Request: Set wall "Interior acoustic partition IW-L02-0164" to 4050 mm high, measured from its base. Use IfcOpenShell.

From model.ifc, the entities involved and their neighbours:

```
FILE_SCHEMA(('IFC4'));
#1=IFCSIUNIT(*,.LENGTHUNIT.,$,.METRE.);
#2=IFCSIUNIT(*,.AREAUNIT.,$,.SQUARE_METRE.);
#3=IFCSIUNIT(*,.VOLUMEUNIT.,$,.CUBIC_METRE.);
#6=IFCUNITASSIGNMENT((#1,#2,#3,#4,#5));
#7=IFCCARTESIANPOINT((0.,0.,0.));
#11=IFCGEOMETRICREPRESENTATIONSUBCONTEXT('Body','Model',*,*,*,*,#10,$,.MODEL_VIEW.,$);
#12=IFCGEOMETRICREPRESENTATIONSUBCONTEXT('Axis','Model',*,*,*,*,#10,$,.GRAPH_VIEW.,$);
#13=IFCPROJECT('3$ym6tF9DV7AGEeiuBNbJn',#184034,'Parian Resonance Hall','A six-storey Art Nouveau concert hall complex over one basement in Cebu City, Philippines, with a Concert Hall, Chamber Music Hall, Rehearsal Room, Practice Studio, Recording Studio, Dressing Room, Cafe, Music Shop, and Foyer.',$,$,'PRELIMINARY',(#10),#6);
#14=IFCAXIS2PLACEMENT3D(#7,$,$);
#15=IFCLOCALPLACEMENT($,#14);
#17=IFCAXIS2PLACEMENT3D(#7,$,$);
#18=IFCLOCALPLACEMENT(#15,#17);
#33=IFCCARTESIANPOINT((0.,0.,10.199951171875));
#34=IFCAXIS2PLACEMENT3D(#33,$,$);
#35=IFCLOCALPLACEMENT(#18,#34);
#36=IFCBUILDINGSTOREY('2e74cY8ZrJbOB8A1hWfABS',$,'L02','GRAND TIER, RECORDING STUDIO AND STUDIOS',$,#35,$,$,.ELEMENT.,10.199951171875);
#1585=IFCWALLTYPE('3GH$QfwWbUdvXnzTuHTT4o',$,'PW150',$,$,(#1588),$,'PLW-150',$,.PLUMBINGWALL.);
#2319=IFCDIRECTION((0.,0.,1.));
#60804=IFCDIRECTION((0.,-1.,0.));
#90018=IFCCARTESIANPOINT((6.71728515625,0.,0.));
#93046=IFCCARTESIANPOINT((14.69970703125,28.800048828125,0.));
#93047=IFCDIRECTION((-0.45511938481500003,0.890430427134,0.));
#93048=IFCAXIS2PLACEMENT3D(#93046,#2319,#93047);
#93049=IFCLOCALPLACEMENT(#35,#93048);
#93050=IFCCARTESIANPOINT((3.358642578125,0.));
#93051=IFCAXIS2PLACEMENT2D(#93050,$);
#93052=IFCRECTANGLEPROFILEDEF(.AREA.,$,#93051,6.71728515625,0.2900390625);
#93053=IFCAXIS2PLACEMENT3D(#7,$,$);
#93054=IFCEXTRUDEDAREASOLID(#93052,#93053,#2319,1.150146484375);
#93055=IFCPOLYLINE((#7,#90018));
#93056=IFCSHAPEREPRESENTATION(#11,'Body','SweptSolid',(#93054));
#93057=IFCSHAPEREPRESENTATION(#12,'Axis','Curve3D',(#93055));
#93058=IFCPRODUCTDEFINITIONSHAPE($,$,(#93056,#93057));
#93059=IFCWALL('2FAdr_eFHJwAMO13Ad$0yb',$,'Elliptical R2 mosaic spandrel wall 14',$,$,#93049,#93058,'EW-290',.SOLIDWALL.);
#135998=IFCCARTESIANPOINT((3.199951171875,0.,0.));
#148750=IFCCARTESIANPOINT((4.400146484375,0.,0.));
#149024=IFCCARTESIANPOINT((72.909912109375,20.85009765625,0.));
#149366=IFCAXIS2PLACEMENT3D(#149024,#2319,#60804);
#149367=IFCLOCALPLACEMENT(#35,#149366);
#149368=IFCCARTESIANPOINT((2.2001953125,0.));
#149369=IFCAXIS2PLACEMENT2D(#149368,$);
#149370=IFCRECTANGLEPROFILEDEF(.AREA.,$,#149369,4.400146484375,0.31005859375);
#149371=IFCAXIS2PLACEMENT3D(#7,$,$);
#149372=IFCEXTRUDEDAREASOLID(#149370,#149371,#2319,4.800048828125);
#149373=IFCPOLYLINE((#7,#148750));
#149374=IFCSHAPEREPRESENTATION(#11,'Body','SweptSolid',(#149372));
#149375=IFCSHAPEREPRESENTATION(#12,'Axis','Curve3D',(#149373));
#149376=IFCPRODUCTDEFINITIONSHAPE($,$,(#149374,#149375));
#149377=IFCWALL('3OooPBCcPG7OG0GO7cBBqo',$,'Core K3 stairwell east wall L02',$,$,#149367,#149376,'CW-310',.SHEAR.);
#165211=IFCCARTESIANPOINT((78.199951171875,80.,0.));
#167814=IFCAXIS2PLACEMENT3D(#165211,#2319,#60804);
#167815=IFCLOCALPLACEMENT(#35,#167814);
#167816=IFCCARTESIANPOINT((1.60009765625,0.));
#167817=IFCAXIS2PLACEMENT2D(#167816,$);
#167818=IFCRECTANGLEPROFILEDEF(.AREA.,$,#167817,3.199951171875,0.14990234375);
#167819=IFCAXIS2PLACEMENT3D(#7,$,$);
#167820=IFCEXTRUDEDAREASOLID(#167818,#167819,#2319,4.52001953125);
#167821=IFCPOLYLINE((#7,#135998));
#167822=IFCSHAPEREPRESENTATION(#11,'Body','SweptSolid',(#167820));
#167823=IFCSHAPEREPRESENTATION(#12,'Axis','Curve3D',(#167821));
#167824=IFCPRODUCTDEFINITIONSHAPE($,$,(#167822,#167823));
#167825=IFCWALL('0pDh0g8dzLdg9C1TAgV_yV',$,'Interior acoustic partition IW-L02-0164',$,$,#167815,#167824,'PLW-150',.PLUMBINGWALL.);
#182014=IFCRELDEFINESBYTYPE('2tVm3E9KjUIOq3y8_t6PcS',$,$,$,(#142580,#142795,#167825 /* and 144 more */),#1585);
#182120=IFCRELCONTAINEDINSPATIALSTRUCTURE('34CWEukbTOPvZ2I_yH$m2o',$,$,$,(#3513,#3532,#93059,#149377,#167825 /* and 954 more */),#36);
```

```python
import ifcopenshell
import ifcopenshell.geom
import ifcopenshell.util.representation
import ifcopenshell.util.shape
import ifcopenshell.util.unit

model = ifcopenshell.open("model.ifc")
unit_scale = ifcopenshell.util.unit.calculate_unit_scale(model)
settings = ifcopenshell.geom.settings()


def volume(element):
    """Net volume in cubic metres, openings subtracted."""
    shape = ifcopenshell.geom.create_shape(settings, element)
    return ifcopenshell.util.shape.get_volume(shape.geometry)


wall = model.by_guid("0pDh0g8dzLdg9C1TAgV_yV")
before = volume(wall)

body = ifcopenshell.util.representation.get_representation(wall, "Model", "Body")
solid = body.Items[0]
old_height = solid.Depth
solid.Depth = 4.05 / unit_scale
after = volume(wall)

print(f"height {old_height:g} -> {solid.Depth:g}, volume {before:.3f} -> {after:.3f} m3")

model.write("model-out.ifc")
```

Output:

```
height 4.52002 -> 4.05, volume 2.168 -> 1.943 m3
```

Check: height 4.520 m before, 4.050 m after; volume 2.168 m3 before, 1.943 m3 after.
